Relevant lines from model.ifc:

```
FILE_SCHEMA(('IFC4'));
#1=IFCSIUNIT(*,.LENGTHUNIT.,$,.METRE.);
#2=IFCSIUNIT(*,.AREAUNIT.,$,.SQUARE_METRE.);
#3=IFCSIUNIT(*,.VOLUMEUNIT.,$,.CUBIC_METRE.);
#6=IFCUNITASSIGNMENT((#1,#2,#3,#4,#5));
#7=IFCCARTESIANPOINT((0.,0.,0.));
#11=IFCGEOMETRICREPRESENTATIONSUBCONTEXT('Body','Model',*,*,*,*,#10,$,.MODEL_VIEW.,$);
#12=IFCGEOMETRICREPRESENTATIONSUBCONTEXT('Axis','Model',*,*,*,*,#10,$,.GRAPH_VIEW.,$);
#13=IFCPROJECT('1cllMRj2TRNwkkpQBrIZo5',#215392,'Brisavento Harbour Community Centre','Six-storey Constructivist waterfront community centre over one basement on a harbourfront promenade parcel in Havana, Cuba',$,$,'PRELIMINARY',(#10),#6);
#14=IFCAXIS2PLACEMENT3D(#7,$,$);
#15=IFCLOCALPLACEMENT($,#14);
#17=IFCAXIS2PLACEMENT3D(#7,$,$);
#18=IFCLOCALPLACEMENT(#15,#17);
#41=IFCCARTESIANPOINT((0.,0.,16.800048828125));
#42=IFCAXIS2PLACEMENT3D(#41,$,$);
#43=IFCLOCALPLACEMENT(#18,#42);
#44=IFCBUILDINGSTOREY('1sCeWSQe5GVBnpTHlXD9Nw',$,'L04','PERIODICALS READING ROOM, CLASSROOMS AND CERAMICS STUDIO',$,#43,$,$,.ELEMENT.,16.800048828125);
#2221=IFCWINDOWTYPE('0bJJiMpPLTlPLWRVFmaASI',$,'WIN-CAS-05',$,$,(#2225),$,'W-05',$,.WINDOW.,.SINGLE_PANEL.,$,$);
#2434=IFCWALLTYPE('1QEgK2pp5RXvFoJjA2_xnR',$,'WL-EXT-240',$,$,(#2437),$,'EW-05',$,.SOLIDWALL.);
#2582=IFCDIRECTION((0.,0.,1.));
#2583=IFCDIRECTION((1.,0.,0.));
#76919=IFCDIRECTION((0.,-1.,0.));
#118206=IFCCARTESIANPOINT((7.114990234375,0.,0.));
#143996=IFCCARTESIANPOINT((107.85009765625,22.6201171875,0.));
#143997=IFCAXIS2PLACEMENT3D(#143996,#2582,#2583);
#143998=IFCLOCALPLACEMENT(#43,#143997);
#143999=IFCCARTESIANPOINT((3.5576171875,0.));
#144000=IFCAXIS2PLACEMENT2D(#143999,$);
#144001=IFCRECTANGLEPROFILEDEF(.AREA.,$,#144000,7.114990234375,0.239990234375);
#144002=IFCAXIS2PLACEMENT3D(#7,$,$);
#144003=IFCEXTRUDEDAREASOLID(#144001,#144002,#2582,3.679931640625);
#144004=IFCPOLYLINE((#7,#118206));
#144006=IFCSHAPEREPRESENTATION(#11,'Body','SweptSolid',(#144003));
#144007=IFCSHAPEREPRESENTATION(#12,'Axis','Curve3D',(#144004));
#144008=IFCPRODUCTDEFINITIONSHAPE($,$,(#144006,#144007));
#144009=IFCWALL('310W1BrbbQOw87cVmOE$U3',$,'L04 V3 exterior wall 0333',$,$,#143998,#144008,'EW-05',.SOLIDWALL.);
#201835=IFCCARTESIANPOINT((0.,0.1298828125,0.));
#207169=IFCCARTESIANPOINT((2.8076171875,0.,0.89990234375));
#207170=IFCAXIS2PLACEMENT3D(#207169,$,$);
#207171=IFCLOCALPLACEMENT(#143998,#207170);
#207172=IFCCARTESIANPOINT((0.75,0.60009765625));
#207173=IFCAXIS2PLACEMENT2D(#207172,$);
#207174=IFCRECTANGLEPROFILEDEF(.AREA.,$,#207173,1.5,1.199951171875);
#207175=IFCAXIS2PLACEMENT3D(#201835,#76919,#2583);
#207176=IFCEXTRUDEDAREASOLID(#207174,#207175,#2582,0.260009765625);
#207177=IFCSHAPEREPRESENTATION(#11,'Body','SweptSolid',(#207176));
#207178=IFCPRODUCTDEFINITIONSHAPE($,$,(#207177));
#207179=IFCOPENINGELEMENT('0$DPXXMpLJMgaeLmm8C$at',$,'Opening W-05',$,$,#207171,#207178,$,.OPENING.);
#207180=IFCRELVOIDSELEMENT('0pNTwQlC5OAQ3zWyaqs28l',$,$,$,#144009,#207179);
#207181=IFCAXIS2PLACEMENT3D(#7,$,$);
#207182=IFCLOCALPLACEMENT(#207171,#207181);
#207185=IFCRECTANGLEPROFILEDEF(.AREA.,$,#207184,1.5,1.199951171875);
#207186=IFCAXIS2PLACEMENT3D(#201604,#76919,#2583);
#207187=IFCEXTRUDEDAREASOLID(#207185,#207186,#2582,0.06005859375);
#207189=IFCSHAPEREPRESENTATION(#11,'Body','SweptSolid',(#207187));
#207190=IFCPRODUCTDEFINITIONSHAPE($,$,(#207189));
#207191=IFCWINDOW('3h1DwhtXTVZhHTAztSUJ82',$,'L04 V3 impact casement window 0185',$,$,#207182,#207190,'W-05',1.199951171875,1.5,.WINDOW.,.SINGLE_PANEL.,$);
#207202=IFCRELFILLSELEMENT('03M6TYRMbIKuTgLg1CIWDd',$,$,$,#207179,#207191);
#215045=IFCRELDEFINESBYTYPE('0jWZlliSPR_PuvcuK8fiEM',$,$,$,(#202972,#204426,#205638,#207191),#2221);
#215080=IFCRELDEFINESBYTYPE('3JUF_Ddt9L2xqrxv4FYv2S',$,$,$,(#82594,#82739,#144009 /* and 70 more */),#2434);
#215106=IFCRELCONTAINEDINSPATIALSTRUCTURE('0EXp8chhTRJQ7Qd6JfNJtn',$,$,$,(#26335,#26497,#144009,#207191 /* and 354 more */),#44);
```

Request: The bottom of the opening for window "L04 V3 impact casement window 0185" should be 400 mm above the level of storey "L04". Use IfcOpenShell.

```python
import numpy as np
import ifcopenshell
import ifcopenshell.api.geometry
import ifcopenshell.geom
import ifcopenshell.util.element
import ifcopenshell.util.placement
import ifcopenshell.util.shape
import ifcopenshell.util.unit

model = ifcopenshell.open("model.ifc")
unit_scale = ifcopenshell.util.unit.calculate_unit_scale(model)

window = model.by_id(207191)
opening = window.FillsVoids[0].RelatingOpeningElement
storey = ifcopenshell.util.element.get_container(window, ifc_class="IfcBuildingStorey")
level = ifcopenshell.util.placement.get_local_placement(storey.ObjectPlacement)[2, 3]

# The opening's origin need not be at the sill, so measure its lowest point.
shape = ifcopenshell.geom.create_shape(ifcopenshell.geom.settings(), opening)
bottom = ifcopenshell.util.shape.get_shape_bottom_elevation(shape, shape.geometry) / unit_scale
dz = level + 0.4 / unit_scale - bottom

shift = np.array([0.0, 0.0, dz])
# The window is placed relative to its opening, so it follows when the opening moves.
matrix = ifcopenshell.util.placement.get_local_placement(opening.ObjectPlacement)
matrix[:3, 3] += shift
ifcopenshell.api.geometry.edit_object_placement(
    model, product=opening, matrix=matrix, is_si=False, should_transform_children=True
)

print(f"moved by {dz * unit_scale:+.3f} m")

model.write("model_updated.ifc")
```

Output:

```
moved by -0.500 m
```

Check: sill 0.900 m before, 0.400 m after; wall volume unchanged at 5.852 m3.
